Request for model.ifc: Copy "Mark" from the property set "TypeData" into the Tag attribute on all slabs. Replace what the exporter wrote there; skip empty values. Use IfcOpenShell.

First a look at what the model holds.

```python
import ifcopenshell
import ifcopenshell.util.element

model = ifcopenshell.open("model.ifc")
print(model.schema)
slabs = model.by_type("IfcSlab")
print(len(slabs), "slabs")
for e in slabs[:8]:
    source = ifcopenshell.util.element.get_pset(e, "TypeData", "Mark")
    target = e.Tag
    print(e.id(), repr(source), repr(target), sep=" | ")
```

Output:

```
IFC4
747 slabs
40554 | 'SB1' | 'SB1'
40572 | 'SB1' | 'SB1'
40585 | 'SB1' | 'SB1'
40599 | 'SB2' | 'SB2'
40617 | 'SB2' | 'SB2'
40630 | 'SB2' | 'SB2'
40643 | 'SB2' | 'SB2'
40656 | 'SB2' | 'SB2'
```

```python
import ifcopenshell
import ifcopenshell.util.element

model = ifcopenshell.open("model.ifc")

count = 0
for e in model.by_type("IfcSlab"):
    value = ifcopenshell.util.element.get_pset(e, "TypeData", "Mark")
    current = e.Tag
    if not value or not value.strip() or current == value:
        continue
    e.Tag = value
    count += 1

print(count, "slabs updated")

model.write("model-out.ifc")
```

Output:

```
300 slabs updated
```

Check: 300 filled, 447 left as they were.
